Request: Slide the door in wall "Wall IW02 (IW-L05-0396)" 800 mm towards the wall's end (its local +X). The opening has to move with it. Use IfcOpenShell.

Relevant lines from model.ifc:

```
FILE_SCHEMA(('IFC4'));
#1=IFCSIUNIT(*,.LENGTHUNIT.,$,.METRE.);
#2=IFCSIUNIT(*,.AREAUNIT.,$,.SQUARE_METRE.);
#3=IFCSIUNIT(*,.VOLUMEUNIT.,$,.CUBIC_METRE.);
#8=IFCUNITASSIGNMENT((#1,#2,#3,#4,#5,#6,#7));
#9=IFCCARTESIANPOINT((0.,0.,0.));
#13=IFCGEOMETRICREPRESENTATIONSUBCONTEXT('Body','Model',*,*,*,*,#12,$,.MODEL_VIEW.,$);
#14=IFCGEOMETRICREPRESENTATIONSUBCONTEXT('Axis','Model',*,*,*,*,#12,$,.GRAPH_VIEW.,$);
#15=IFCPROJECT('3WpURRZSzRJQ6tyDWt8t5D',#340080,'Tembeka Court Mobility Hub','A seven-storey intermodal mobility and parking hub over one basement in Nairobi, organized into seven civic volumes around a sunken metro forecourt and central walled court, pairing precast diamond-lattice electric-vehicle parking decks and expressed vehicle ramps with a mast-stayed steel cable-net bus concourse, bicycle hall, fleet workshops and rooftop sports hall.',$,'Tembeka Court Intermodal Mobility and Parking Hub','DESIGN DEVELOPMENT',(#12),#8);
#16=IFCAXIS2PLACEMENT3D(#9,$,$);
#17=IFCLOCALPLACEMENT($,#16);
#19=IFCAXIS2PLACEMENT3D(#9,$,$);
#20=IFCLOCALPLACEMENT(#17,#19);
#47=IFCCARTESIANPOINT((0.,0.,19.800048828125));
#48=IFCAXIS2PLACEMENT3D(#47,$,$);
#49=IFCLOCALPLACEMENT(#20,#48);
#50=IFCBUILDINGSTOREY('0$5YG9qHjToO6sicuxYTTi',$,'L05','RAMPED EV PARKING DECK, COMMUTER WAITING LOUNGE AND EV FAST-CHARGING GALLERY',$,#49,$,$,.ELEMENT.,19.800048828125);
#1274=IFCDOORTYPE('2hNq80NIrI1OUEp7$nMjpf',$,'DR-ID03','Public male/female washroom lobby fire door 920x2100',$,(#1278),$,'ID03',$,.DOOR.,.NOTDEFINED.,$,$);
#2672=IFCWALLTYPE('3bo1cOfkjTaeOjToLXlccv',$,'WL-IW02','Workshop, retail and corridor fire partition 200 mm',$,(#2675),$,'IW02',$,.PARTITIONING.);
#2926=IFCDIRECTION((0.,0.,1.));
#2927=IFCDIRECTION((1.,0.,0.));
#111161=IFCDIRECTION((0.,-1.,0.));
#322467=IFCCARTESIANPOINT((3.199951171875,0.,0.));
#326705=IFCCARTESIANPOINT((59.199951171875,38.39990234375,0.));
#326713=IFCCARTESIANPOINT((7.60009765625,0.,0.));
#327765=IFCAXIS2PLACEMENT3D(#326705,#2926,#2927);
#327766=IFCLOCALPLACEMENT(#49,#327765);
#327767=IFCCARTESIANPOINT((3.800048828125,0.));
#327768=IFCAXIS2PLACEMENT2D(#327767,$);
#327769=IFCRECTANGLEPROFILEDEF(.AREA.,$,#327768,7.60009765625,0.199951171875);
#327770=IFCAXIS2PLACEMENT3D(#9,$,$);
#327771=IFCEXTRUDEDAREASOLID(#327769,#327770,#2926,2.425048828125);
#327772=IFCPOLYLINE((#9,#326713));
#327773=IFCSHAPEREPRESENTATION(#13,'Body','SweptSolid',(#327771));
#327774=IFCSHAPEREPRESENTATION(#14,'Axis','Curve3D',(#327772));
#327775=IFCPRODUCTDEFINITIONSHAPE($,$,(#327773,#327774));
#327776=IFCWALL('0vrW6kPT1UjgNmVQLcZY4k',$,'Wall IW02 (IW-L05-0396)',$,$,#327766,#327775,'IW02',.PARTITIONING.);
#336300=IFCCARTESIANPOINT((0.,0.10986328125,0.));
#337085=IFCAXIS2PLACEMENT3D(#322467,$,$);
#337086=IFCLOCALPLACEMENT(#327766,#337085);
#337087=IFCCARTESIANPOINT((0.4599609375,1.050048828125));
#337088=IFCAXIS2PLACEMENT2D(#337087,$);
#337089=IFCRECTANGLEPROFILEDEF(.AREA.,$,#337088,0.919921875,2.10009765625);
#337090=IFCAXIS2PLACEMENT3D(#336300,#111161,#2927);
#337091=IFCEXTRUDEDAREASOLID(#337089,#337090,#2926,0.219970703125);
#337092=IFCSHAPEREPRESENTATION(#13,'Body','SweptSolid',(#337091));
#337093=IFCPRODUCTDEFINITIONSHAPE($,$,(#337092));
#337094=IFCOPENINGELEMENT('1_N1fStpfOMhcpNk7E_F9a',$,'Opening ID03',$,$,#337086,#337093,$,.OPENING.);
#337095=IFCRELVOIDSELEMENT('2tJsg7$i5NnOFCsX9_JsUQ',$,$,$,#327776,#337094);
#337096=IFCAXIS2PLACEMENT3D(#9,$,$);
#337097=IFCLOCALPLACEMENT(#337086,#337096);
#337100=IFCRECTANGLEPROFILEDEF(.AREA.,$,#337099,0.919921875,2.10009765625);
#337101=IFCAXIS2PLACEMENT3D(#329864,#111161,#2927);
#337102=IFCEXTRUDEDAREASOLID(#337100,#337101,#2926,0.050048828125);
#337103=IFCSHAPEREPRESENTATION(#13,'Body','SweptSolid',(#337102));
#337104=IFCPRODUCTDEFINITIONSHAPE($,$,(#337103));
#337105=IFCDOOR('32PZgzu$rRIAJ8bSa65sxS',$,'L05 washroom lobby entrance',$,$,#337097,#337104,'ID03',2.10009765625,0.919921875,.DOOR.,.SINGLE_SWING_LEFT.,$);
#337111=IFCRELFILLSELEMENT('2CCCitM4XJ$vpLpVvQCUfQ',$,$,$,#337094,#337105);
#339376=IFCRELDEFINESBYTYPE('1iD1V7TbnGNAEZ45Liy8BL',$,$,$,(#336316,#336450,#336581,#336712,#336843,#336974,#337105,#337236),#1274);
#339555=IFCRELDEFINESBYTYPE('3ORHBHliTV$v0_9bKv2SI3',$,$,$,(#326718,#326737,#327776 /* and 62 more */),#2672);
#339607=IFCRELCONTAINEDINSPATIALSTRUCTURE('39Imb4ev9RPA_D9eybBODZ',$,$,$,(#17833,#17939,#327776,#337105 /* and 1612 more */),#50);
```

```python
import ifcopenshell
import ifcopenshell.api.geometry
import ifcopenshell.util.placement

model = ifcopenshell.open("model.ifc")

door = model.by_id(337105)
opening = door.FillsVoids[0].RelatingOpeningElement
wall = opening.VoidsElements[0].RelatingBuildingElement

wall_matrix = ifcopenshell.util.placement.get_local_placement(wall.ObjectPlacement)
shift = wall_matrix[:3, 0] * 0.8
before = ifcopenshell.util.placement.get_local_placement(door.ObjectPlacement)[:3, 3].copy()

# The door is placed relative to its opening, so it follows when the opening moves.
matrix = ifcopenshell.util.placement.get_local_placement(opening.ObjectPlacement)
matrix[:3, 3] += shift
ifcopenshell.api.geometry.edit_object_placement(
    model, product=opening, matrix=matrix, is_si=False, should_transform_children=True
)

after = ifcopenshell.util.placement.get_local_placement(door.ObjectPlacement)[:3, 3]
print("door moved by", (after - before).round(3) + 0.0)

model.write("model-out.ifc")
```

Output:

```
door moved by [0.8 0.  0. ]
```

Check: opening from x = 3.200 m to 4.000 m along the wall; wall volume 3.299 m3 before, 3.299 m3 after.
